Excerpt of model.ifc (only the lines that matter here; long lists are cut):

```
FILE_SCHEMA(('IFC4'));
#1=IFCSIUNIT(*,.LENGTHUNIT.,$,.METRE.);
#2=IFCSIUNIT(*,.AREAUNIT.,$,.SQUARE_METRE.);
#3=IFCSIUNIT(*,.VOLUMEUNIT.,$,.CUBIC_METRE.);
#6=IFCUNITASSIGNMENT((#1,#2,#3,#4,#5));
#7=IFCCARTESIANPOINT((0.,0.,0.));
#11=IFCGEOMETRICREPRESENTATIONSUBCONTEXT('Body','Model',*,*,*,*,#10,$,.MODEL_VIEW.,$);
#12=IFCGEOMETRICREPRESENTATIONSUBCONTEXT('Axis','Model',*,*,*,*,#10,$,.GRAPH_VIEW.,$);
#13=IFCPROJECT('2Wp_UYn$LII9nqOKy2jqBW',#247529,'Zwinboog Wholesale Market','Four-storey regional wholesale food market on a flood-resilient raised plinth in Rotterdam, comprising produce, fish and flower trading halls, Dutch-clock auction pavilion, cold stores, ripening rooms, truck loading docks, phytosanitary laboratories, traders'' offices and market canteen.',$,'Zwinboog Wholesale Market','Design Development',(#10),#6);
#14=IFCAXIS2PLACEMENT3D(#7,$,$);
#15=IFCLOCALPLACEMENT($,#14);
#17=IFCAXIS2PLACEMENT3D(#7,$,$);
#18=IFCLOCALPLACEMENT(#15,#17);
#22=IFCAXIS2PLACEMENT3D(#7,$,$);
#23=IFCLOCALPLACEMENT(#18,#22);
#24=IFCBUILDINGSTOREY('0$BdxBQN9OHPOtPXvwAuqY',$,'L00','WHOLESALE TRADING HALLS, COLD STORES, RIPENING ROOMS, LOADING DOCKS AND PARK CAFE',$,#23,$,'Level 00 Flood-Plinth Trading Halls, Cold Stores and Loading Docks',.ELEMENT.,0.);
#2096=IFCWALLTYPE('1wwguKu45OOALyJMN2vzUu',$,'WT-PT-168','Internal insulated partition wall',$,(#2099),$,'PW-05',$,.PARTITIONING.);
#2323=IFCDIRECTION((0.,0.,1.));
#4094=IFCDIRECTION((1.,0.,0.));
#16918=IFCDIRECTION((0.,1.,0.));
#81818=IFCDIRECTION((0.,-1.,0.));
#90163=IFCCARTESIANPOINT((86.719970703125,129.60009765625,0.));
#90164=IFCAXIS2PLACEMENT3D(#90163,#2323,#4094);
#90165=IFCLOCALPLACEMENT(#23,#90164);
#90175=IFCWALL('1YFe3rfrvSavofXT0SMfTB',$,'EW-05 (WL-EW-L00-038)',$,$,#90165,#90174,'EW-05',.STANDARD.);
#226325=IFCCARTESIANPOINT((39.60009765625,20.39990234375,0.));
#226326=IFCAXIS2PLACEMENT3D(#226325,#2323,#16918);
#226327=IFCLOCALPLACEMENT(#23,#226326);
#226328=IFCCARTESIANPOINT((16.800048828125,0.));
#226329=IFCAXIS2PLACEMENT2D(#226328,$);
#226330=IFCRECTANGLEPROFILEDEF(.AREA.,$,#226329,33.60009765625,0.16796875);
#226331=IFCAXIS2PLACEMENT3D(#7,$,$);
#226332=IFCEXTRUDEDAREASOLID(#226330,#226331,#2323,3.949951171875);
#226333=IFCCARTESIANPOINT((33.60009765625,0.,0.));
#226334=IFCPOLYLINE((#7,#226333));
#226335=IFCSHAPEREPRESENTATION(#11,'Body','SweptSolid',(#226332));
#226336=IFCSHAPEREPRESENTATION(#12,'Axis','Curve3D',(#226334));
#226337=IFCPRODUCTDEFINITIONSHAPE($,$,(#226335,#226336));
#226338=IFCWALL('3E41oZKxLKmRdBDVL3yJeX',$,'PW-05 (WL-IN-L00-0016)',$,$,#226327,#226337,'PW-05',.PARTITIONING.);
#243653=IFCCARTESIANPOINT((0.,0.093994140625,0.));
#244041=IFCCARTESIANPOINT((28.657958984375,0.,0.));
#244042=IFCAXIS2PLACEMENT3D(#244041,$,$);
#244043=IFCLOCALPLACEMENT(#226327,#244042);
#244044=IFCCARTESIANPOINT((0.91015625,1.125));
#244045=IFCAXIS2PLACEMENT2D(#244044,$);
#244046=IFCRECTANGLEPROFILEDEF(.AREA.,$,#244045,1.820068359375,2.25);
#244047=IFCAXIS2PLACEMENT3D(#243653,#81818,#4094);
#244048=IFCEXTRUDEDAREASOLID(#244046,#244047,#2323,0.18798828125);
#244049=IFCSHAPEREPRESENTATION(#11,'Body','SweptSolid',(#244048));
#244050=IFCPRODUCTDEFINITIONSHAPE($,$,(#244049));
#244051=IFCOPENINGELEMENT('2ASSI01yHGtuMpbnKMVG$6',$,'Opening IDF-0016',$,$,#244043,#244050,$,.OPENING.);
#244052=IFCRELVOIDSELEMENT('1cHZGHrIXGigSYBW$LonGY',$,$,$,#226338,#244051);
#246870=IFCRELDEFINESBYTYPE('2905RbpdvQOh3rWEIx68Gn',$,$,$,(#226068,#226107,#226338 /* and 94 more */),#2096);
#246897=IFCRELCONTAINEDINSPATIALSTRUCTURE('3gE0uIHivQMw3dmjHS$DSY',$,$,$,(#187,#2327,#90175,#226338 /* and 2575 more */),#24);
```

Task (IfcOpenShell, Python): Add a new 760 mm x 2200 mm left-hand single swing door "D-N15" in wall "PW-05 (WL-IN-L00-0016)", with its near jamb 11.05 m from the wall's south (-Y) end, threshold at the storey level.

```python
import numpy as np
import ifcopenshell
import ifcopenshell.api.feature
import ifcopenshell.api.geometry
import ifcopenshell.api.root
import ifcopenshell.api.spatial
import ifcopenshell.geom
import ifcopenshell.util.element
import ifcopenshell.util.placement
import ifcopenshell.util.representation
import ifcopenshell.util.shape
import ifcopenshell.util.unit

model = ifcopenshell.open("model.ifc")
unit_scale = ifcopenshell.util.unit.calculate_unit_scale(model)
settings = ifcopenshell.geom.settings()


def volume(element):
    """Net volume in cubic metres, openings subtracted."""
    shape = ifcopenshell.geom.create_shape(settings, element)
    return ifcopenshell.util.shape.get_volume(shape.geometry)


wall = model.by_guid("3E41oZKxLKmRdBDVL3yJeX")
storey = ifcopenshell.util.element.get_container(wall, ifc_class="IfcBuildingStorey")
context = ifcopenshell.util.representation.get_context(model, "Model", "Body", "MODEL_VIEW")
before = volume(wall)

width, height, from_end, sill = 0.76, 2.2, 11.05, 0.0  # metres

# The wall runs along its own X axis, and the end named is its -X end.
wall_shape = ifcopenshell.geom.create_shape(settings, wall)
x, y, z = ifcopenshell.util.shape.get_vertices(wall_shape.geometry).T
start = x.min() + from_end
face, thickness = float(y.min()), float(y.max() - y.min())
wall_matrix = ifcopenshell.util.placement.get_local_placement(wall.ObjectPlacement)
level = ifcopenshell.util.placement.get_local_placement(storey.ObjectPlacement)[2, 3]


def in_wall(x, y):
    """Placement at x, y metres in the wall's axes, at sill height."""
    matrix = wall_matrix.copy()
    matrix[:, 3] = wall_matrix @ np.array([x / unit_scale, y / unit_scale, 0.0, 1.0])
    matrix[2, 3] = level + sill / unit_scale
    return matrix


# Opening: a box that overshoots both wall faces by 50 mm.
opening = ifcopenshell.api.root.create_entity(model, ifc_class="IfcOpeningElement", predefined_type="OPENING")
box = ifcopenshell.api.geometry.add_wall_representation(
    model, context=context, length=width, height=height, thickness=thickness + 0.1
)
ifcopenshell.api.geometry.assign_representation(model, product=opening, representation=box)
ifcopenshell.api.geometry.edit_object_placement(model, product=opening, matrix=in_wall(start, face - 0.05), is_si=False)
ifcopenshell.api.feature.add_feature(model, feature=opening, element=wall)

door = ifcopenshell.api.root.create_entity(model, ifc_class="IfcDoor", name="D-N15", predefined_type="DOOR")
door.OverallWidth, door.OverallHeight = width / unit_scale, height / unit_scale
door.OperationType = "SINGLE_SWING_LEFT"
body = ifcopenshell.api.geometry.add_door_representation(
    model,
    context=context,
    overall_width=door.OverallWidth,
    overall_height=door.OverallHeight,
    operation_type="SINGLE_SWING_LEFT",
    lining_properties={"LiningDepth": thickness / unit_scale, "ThresholdDepth": thickness / unit_scale},
)
ifcopenshell.api.geometry.assign_representation(model, product=door, representation=body)
ifcopenshell.api.spatial.assign_container(model, products=[door], relating_structure=storey)
ifcopenshell.api.feature.add_filling(model, opening=opening, element=door)

# The lining spans the wall, so the door starts at the wall face.
ifcopenshell.api.geometry.edit_object_placement(model, product=door, matrix=in_wall(start, face), is_si=False)

after = volume(wall)

print(f"wall volume {before:.3f} -> {after:.3f} m3")

model.write("model-out.ifc")
```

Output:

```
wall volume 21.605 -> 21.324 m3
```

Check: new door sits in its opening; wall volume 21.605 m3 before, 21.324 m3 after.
